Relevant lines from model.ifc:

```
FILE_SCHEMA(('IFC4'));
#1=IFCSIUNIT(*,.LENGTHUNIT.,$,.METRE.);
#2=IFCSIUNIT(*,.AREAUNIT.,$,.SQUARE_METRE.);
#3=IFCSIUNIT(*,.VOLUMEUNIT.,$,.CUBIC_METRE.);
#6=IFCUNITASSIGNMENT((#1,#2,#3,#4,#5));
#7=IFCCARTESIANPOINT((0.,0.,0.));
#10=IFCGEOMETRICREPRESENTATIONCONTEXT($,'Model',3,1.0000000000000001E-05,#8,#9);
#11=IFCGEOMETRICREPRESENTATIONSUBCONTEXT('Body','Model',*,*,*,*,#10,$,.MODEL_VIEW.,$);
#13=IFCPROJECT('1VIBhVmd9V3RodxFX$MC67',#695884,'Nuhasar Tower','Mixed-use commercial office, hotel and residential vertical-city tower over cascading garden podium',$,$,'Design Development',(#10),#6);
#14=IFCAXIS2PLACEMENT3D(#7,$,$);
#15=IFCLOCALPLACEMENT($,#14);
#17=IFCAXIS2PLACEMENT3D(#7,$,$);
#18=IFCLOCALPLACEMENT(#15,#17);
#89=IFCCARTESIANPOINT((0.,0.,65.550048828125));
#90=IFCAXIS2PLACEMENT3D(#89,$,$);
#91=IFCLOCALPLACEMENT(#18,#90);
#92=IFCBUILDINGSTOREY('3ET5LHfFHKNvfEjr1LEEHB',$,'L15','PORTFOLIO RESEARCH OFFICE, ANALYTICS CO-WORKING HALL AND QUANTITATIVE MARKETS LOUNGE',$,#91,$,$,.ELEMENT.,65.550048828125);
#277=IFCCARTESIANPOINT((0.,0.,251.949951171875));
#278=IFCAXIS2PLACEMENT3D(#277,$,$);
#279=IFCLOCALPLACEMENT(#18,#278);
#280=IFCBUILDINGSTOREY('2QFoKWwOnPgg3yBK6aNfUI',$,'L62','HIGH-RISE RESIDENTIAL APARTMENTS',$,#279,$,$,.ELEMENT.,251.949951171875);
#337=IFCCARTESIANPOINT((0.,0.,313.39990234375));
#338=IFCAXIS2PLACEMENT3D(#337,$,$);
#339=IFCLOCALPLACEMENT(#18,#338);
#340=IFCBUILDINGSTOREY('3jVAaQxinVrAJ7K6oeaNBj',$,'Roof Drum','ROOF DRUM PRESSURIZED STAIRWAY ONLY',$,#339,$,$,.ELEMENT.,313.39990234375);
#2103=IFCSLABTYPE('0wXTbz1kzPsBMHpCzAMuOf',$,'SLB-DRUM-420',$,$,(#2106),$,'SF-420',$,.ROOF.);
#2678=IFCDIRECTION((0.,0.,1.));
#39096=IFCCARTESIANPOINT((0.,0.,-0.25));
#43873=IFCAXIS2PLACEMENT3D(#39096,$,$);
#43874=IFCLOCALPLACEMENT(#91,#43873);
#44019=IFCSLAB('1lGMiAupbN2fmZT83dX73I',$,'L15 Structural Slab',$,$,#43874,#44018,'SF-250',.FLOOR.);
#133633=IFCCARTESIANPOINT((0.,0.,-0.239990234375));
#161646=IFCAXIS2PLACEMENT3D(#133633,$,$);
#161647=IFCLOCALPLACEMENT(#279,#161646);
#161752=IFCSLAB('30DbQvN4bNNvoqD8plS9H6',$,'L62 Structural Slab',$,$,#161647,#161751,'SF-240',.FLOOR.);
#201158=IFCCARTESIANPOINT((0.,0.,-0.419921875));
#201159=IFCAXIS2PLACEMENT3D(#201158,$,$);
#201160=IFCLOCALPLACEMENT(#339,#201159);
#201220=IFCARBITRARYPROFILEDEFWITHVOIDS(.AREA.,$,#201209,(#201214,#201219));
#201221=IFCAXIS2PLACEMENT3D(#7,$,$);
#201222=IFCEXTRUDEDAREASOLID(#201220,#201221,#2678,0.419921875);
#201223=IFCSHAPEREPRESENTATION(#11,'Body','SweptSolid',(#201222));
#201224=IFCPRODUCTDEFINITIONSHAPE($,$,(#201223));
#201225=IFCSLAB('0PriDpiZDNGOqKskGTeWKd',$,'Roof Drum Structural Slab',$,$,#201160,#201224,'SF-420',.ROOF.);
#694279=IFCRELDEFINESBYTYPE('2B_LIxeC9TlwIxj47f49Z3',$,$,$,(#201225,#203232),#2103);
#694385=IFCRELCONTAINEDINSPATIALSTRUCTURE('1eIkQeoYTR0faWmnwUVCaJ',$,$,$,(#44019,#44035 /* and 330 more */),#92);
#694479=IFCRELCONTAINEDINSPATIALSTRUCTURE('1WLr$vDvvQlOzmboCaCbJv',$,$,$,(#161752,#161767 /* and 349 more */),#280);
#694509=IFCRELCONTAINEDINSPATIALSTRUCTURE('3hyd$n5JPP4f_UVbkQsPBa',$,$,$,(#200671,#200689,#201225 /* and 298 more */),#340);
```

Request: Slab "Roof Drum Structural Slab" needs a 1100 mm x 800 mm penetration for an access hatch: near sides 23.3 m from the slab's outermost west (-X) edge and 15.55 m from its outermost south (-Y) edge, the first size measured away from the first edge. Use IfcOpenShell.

```python
import numpy as np
import ifcopenshell
import ifcopenshell.api.feature
import ifcopenshell.api.geometry
import ifcopenshell.api.root
import ifcopenshell.geom
import ifcopenshell.util.placement
import ifcopenshell.util.representation
import ifcopenshell.util.shape
import ifcopenshell.util.unit

model = ifcopenshell.open("model.ifc")
unit_scale = ifcopenshell.util.unit.calculate_unit_scale(model)
settings = ifcopenshell.geom.settings()


def volume(element):
    """Net volume in cubic metres, openings subtracted."""
    shape = ifcopenshell.geom.create_shape(settings, element)
    return ifcopenshell.util.shape.get_volume(shape.geometry)


slab = model.by_id(201225)
before = volume(slab)

# Extent in the slab's own axes, in metres. The edges named are its -X and -Y sides.
slab_shape = ifcopenshell.geom.create_shape(settings, slab)
vertices = ifcopenshell.util.shape.get_vertices(slab_shape.geometry)
x_min, y_min, bottom = vertices.min(axis=0)
top = vertices[:, 2].max()

opening = ifcopenshell.api.root.create_entity(model, ifc_class="IfcOpeningElement", name="Access hatch opening", predefined_type="OPENING")
context = ifcopenshell.util.representation.get_context(model, "Model", "Body", "MODEL_VIEW")
width, depth = 1.1, 0.8
outline = [(0.0, 0.0), (width, 0.0), (width, depth), (0.0, depth), (0.0, 0.0)]
# Overshoot both faces by 50 mm so the cut is clean.
shape = ifcopenshell.api.geometry.add_slab_representation(
    model, context=context, depth=top - bottom + 0.1, polyline=outline
)
ifcopenshell.api.geometry.assign_representation(model, product=opening, representation=shape)

matrix = ifcopenshell.util.placement.get_local_placement(slab.ObjectPlacement)
matrix[:, 3] = matrix @ np.append(np.array([x_min + 23.3, y_min + 15.55, bottom - 0.05]) / unit_scale, 1.0)
ifcopenshell.api.geometry.edit_object_placement(model, product=opening, matrix=matrix, is_si=False)
ifcopenshell.api.feature.add_feature(model, feature=opening, element=slab)

after = volume(slab)

print(f"slab volume {before:.3f} -> {after:.3f} m3")

model.write("model-out.ifc")
```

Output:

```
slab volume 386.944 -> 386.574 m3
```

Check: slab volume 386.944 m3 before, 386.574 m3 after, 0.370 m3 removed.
